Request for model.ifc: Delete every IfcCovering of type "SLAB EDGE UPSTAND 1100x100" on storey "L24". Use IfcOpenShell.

First a look at what the model holds.

```python
import ifcopenshell
import ifcopenshell.util.element

model = ifcopenshell.open("model.ifc")
print(model.schema)
storey = next(s for s in model.by_type("IfcBuildingStorey") if s.Name == "L24")
coverings = [e for e in ifcopenshell.util.element.get_decomposition(storey) if e.is_a("IfcCovering")]
seen = {}
for e in coverings:
    element_type = ifcopenshell.util.element.get_type(e)
    name = element_type.Name if element_type not in (None, e) else None
    seen[name] = seen.get(name, 0) + 1
for name, count in sorted(seen.items(), key=str):
    print(count, "x", name)
```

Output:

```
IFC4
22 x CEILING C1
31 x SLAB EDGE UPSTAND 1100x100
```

```python
import ifcopenshell
import ifcopenshell.api.root
import ifcopenshell.util.element

model = ifcopenshell.open("model.ifc")

storey = next(s for s in model.by_type("IfcBuildingStorey") if s.Name == "L24")
coverings = [e for e in ifcopenshell.util.element.get_decomposition(storey) if e.is_a("IfcCovering")]
targets = [e for e in coverings if (t := ifcopenshell.util.element.get_type(e)) not in (None, e) and t.Name == "SLAB EDGE UPSTAND 1100x100"]

for e in targets:
    ifcopenshell.api.root.remove_product(model, product=e)
print(len(targets), "removed")

model.write("model_edited.ifc")
```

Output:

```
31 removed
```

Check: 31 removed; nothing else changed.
